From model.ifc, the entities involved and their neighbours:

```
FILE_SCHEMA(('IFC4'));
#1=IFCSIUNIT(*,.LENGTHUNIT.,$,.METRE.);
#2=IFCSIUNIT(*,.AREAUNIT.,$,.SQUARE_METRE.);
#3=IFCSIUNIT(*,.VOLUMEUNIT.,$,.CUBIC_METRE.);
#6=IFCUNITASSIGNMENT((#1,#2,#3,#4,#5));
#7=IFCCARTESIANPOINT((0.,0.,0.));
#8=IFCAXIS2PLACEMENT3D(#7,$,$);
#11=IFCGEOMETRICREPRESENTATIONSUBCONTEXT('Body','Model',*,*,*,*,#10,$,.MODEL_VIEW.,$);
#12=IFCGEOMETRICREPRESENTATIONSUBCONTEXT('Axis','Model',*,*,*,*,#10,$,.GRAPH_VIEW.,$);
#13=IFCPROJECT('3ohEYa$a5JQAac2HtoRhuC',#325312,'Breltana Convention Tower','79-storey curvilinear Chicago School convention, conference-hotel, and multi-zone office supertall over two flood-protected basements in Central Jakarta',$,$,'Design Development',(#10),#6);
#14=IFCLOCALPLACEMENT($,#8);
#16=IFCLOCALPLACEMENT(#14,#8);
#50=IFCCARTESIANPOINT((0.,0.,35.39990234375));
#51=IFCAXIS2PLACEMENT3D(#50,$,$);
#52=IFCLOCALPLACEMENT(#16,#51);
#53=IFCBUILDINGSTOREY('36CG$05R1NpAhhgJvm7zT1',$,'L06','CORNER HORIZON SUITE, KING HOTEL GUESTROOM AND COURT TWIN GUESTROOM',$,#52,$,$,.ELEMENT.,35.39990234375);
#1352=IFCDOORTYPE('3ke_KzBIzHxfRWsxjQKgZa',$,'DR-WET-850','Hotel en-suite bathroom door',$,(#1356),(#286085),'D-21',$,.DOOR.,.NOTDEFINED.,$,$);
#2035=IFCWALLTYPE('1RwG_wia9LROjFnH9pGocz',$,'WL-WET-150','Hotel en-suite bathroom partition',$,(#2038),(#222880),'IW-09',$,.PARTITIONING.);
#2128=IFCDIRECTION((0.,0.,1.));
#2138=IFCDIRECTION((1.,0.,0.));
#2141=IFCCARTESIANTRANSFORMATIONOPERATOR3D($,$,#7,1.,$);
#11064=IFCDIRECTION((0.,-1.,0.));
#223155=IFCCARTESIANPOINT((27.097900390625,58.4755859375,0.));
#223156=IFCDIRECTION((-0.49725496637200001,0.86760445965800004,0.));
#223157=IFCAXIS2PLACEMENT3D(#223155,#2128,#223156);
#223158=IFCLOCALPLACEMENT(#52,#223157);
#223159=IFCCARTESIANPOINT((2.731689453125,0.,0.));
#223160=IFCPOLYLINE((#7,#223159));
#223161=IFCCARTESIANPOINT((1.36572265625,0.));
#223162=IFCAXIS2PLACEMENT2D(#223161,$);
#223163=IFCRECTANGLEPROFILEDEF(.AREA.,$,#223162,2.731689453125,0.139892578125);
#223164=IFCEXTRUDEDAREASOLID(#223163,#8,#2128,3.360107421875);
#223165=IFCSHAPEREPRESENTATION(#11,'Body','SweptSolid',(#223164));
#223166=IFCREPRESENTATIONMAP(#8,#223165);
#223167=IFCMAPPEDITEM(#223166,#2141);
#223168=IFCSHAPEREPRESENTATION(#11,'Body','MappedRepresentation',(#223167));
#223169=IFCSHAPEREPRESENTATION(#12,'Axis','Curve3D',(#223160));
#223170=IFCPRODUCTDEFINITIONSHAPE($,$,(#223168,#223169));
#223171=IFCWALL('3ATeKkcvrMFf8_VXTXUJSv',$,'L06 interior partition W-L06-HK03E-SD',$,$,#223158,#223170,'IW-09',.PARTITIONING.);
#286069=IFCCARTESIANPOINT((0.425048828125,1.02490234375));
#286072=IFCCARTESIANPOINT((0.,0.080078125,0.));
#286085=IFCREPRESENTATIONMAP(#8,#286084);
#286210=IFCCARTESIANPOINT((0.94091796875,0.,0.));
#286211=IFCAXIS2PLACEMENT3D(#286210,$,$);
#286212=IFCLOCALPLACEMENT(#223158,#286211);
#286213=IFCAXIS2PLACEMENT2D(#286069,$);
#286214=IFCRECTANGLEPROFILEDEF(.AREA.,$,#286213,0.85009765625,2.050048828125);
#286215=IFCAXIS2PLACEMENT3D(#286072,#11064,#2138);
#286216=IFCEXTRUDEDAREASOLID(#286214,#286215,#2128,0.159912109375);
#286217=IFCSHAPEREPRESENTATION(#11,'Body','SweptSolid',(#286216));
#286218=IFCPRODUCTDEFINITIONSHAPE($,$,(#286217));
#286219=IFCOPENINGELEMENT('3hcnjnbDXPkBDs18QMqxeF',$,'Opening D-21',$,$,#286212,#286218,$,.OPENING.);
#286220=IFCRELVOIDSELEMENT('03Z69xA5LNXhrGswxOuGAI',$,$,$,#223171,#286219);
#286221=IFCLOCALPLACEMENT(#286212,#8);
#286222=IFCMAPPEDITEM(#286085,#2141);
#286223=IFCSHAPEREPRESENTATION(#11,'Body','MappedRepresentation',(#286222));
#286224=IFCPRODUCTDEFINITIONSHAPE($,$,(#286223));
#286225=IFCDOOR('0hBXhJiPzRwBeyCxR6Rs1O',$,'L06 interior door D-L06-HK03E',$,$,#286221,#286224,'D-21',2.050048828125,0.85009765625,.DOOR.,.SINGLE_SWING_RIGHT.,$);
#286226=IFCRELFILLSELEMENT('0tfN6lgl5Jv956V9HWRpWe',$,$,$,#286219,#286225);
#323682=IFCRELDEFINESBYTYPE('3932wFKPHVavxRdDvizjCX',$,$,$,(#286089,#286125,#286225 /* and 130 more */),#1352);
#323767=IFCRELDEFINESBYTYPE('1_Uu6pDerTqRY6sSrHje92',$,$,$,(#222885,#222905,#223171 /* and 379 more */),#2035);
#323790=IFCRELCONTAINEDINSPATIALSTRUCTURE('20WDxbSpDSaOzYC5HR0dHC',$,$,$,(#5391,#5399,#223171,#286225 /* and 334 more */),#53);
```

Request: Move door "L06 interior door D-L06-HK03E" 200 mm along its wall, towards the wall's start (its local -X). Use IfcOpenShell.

```python
import ifcopenshell
import ifcopenshell.api.geometry
import ifcopenshell.util.placement
import ifcopenshell.util.unit

model = ifcopenshell.open("model.ifc")
unit_scale = ifcopenshell.util.unit.calculate_unit_scale(model)

door = model.by_guid("0hBXhJiPzRwBeyCxR6Rs1O")
opening = door.FillsVoids[0].RelatingOpeningElement
wall = opening.VoidsElements[0].RelatingBuildingElement

wall_matrix = ifcopenshell.util.placement.get_local_placement(wall.ObjectPlacement)
shift = wall_matrix[:3, 0] * -0.2 / unit_scale
before = ifcopenshell.util.placement.get_local_placement(door.ObjectPlacement)[:3, 3].copy()

# The door is placed relative to its opening, so it follows when the opening moves.
matrix = ifcopenshell.util.placement.get_local_placement(opening.ObjectPlacement)
matrix[:3, 3] += shift
ifcopenshell.api.geometry.edit_object_placement(
    model, product=opening, matrix=matrix, is_si=False, should_transform_children=True
)

after = ifcopenshell.util.placement.get_local_placement(door.ObjectPlacement)[:3, 3]
print("door moved by", (after - before).round(3) + 0.0)

model.write("model-out.ifc")
```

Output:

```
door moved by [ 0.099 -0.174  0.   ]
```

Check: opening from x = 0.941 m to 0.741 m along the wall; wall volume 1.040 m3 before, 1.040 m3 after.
